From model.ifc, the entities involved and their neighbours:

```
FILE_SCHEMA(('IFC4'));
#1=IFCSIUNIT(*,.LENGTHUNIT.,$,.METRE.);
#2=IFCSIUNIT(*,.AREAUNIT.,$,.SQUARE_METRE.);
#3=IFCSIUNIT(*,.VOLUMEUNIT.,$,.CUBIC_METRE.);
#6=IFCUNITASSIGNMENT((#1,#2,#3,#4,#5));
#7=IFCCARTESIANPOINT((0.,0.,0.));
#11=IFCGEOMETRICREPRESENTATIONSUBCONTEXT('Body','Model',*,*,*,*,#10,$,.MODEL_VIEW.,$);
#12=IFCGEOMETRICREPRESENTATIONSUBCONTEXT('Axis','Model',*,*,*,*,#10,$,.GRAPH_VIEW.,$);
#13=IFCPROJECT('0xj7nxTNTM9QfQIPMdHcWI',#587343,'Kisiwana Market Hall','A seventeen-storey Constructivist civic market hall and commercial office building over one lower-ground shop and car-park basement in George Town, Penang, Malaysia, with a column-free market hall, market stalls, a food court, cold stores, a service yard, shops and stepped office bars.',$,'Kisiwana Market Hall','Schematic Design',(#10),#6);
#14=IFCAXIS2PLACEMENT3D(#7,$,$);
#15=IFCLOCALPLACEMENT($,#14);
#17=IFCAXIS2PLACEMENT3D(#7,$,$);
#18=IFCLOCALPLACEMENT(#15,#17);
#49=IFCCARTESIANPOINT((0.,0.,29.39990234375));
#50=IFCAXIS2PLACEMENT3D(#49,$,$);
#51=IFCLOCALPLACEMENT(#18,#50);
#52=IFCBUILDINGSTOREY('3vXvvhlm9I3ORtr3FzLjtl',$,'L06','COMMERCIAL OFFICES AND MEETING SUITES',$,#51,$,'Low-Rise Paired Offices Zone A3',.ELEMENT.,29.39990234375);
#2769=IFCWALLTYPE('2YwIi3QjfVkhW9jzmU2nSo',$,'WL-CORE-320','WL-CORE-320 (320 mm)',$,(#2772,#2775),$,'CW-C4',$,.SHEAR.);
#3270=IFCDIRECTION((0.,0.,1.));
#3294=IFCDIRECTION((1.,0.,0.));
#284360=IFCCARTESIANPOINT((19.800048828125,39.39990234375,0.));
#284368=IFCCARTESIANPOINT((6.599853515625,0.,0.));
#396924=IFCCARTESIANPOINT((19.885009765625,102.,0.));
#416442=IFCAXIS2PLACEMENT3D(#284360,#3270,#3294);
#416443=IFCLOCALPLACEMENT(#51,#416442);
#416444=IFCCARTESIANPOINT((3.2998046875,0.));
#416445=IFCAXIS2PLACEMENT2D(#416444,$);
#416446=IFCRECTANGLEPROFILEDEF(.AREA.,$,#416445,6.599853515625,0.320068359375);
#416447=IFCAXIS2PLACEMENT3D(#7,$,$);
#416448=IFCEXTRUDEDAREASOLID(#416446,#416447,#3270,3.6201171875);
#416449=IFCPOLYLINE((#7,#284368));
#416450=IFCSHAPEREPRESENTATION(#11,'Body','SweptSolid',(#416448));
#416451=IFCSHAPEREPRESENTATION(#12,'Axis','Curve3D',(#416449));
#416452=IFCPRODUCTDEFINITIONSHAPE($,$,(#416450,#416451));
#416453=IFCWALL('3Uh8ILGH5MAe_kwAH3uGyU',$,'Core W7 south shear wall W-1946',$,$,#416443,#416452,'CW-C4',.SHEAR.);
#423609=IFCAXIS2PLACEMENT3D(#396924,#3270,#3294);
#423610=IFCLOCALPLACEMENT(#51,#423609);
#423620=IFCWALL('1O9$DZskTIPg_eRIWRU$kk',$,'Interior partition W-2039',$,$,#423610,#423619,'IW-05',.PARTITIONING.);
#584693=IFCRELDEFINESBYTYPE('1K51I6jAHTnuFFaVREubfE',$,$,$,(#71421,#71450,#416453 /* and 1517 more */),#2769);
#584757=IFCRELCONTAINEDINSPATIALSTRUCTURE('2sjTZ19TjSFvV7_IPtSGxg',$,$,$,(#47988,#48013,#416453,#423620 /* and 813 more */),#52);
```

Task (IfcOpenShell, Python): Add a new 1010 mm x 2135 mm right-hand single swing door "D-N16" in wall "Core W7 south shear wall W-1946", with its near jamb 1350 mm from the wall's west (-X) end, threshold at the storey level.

```python
import numpy as np
import ifcopenshell
import ifcopenshell.api.feature
import ifcopenshell.api.geometry
import ifcopenshell.api.root
import ifcopenshell.api.spatial
import ifcopenshell.geom
import ifcopenshell.util.element
import ifcopenshell.util.placement
import ifcopenshell.util.representation
import ifcopenshell.util.shape
import ifcopenshell.util.unit

model = ifcopenshell.open("model.ifc")
unit_scale = ifcopenshell.util.unit.calculate_unit_scale(model)
settings = ifcopenshell.geom.settings()


def volume(element):
    """Net volume in cubic metres, openings subtracted."""
    shape = ifcopenshell.geom.create_shape(settings, element)
    return ifcopenshell.util.shape.get_volume(shape.geometry)


wall = model.by_guid("3Uh8ILGH5MAe_kwAH3uGyU")
storey = ifcopenshell.util.element.get_container(wall, ifc_class="IfcBuildingStorey")
context = ifcopenshell.util.representation.get_context(model, "Model", "Body", "MODEL_VIEW")
before = volume(wall)

width, height, from_end, sill = 1.01, 2.135, 1.35, 0.0  # metres

# The wall runs along its own X axis, and the end named is its -X end.
wall_shape = ifcopenshell.geom.create_shape(settings, wall)
x, y, z = ifcopenshell.util.shape.get_vertices(wall_shape.geometry).T
start = x.min() + from_end
face, thickness = float(y.min()), float(y.max() - y.min())
wall_matrix = ifcopenshell.util.placement.get_local_placement(wall.ObjectPlacement)
level = ifcopenshell.util.placement.get_local_placement(storey.ObjectPlacement)[2, 3]


def in_wall(x, y):
    """Placement at x, y metres in the wall's axes, at sill height."""
    matrix = wall_matrix.copy()
    matrix[:, 3] = wall_matrix @ np.array([x / unit_scale, y / unit_scale, 0.0, 1.0])
    matrix[2, 3] = level + sill / unit_scale
    return matrix


# Opening: a box that overshoots both wall faces by 50 mm.
opening = ifcopenshell.api.root.create_entity(model, ifc_class="IfcOpeningElement", predefined_type="OPENING")
box = ifcopenshell.api.geometry.add_wall_representation(
    model, context=context, length=width, height=height, thickness=thickness + 0.1
)
ifcopenshell.api.geometry.assign_representation(model, product=opening, representation=box)
ifcopenshell.api.geometry.edit_object_placement(model, product=opening, matrix=in_wall(start, face - 0.05), is_si=False)
ifcopenshell.api.feature.add_feature(model, feature=opening, element=wall)

door = ifcopenshell.api.root.create_entity(model, ifc_class="IfcDoor", name="D-N16", predefined_type="DOOR")
door.OverallWidth, door.OverallHeight = width / unit_scale, height / unit_scale
door.OperationType = "SINGLE_SWING_RIGHT"
body = ifcopenshell.api.geometry.add_door_representation(
    model,
    context=context,
    overall_width=door.OverallWidth,
    overall_height=door.OverallHeight,
    operation_type="SINGLE_SWING_RIGHT",
    lining_properties={"LiningDepth": thickness / unit_scale, "ThresholdDepth": thickness / unit_scale},
)
ifcopenshell.api.geometry.assign_representation(model, product=door, representation=body)
ifcopenshell.api.spatial.assign_container(model, products=[door], relating_structure=storey)
ifcopenshell.api.feature.add_filling(model, opening=opening, element=door)

# The lining spans the wall, so the door starts at the wall face.
ifcopenshell.api.geometry.edit_object_placement(model, product=door, matrix=in_wall(start, face), is_si=False)

after = volume(wall)

print(f"wall volume {before:.3f} -> {after:.3f} m3")

model.write("model_v2.ifc")
```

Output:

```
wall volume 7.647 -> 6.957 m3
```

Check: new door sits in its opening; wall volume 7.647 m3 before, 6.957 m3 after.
